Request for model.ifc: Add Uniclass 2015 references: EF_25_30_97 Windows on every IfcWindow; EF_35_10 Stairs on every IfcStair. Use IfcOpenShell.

First a look at what the model holds.

```python
import ifcopenshell

model = ifcopenshell.open("model.ifc")
print(model.schema)
print("classifications:", [c.Name for c in model.by_type("IfcClassification")])
for ifc_class in ("IfcDoor", "IfcRoof", "IfcStair", "IfcWall", "IfcWindow"):
    print(ifc_class, len(model.by_type(ifc_class)))
```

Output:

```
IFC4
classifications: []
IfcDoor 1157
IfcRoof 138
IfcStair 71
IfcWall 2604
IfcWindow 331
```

```python
import ifcopenshell
import ifcopenshell.api.classification

model = ifcopenshell.open("model.ifc")

system = ifcopenshell.api.classification.add_classification(model, classification="Uniclass 2015")

codes = {
    "IfcWindow": ("EF_25_30_97", "Windows"),
    "IfcStair": ("EF_35_10", "Stairs"),
}
for ifc_class, (code, name) in codes.items():
    products = model.by_type(ifc_class)
    ifcopenshell.api.classification.add_reference(
        model, products=products, classification=system, identification=code, name=name
    )
    print(code, len(products))

model.write("model_rev.ifc")
```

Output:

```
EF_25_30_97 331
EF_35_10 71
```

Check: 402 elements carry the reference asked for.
